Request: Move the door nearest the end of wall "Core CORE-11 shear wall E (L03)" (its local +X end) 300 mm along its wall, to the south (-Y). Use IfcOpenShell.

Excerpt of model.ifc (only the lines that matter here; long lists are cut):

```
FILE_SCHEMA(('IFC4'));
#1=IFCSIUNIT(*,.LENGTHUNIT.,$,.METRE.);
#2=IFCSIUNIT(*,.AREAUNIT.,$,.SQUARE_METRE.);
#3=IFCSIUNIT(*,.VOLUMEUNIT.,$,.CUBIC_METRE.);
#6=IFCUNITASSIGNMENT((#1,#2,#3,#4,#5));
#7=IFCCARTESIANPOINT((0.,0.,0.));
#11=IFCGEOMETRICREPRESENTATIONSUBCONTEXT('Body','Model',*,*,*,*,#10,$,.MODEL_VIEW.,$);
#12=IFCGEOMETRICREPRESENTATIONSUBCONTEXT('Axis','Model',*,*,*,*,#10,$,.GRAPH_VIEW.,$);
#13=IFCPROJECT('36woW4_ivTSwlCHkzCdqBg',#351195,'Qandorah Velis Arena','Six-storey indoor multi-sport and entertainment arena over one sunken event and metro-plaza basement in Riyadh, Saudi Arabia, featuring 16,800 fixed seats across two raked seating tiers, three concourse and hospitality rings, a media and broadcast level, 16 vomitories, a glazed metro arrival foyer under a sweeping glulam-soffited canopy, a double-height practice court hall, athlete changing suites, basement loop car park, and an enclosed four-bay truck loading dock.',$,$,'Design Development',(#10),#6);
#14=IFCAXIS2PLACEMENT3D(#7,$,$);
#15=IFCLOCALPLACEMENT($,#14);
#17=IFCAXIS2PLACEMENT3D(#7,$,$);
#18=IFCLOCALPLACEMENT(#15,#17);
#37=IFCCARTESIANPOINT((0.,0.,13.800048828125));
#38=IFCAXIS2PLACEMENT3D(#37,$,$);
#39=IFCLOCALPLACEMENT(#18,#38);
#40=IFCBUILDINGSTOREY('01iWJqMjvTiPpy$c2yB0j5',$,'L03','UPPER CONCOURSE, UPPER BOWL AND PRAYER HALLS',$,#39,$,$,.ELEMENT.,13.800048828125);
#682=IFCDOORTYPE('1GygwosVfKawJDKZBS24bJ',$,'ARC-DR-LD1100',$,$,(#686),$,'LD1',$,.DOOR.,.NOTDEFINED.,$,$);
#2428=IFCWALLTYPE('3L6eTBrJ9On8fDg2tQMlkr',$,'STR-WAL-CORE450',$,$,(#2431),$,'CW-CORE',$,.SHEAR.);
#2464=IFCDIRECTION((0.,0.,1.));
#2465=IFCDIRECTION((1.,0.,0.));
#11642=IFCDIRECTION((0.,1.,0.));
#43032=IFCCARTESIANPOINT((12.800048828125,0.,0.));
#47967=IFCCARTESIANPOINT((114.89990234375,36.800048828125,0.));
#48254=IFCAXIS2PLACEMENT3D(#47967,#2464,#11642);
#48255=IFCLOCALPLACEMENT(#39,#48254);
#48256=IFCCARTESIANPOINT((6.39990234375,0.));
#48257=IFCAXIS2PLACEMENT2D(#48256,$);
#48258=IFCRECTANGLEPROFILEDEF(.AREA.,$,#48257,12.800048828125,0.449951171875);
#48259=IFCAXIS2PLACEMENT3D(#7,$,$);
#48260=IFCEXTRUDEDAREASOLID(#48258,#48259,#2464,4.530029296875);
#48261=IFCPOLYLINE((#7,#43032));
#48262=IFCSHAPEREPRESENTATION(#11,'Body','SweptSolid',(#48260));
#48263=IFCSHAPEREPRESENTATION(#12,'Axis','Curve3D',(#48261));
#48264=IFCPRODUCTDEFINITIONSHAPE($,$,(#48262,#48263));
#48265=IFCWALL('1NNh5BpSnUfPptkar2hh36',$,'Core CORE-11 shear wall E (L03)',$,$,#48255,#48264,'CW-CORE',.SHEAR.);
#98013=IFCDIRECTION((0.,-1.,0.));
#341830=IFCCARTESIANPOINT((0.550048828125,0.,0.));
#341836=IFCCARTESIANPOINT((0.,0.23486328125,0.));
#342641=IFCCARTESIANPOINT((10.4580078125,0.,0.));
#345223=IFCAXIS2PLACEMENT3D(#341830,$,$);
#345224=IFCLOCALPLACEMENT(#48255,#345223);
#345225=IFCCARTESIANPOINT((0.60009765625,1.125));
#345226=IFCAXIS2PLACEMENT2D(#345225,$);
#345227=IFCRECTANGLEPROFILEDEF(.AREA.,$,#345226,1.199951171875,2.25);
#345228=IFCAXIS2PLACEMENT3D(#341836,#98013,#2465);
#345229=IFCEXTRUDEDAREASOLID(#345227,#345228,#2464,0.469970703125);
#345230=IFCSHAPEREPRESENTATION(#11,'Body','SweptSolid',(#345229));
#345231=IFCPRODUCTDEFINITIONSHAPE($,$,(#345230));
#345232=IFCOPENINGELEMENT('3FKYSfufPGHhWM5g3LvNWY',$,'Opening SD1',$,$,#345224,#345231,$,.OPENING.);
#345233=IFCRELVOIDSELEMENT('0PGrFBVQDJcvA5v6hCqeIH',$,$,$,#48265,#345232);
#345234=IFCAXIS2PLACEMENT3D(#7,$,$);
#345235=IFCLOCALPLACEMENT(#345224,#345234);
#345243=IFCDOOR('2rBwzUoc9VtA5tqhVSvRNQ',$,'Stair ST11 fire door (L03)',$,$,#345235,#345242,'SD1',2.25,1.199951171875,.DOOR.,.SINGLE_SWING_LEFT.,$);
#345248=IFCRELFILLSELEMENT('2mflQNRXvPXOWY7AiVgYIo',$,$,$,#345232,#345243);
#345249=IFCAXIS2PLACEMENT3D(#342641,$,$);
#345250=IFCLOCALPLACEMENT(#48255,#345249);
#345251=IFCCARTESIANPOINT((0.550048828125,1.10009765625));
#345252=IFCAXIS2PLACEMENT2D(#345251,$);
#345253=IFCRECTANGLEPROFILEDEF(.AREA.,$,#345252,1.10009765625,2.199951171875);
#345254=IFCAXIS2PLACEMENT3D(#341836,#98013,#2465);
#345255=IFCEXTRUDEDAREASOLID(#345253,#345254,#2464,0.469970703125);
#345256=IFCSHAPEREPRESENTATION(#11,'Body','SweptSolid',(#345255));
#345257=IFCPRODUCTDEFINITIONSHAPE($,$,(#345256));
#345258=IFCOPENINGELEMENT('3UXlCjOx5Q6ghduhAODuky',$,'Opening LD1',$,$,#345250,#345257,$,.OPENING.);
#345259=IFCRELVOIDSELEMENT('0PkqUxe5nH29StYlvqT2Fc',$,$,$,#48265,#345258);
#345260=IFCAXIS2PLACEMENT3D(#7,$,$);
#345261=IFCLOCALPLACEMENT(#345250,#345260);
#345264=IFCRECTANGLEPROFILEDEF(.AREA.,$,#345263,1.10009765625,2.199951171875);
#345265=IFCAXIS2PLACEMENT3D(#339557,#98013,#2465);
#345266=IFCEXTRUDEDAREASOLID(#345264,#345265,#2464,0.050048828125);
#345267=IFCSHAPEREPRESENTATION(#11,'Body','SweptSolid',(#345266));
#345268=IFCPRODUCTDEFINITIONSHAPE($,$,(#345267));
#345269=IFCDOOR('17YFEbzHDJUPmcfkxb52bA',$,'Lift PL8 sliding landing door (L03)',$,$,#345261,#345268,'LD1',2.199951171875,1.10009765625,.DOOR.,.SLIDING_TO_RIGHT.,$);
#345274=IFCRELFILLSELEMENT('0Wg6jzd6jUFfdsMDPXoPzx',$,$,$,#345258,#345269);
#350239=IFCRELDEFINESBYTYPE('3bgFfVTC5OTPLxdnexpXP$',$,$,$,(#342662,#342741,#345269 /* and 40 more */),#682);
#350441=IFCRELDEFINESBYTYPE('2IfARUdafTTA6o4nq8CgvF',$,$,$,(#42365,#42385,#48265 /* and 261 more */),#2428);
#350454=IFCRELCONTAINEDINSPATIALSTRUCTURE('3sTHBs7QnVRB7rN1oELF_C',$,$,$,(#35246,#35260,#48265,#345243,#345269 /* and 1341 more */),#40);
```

```python
import ifcopenshell
import ifcopenshell.api.geometry
import ifcopenshell.util.placement

model = ifcopenshell.open("model.ifc")

door = model.by_id(345269)
opening = door.FillsVoids[0].RelatingOpeningElement
wall = opening.VoidsElements[0].RelatingBuildingElement

wall_matrix = ifcopenshell.util.placement.get_local_placement(wall.ObjectPlacement)
shift = wall_matrix[:3, 0] * -0.3
before = ifcopenshell.util.placement.get_local_placement(door.ObjectPlacement)[:3, 3].copy()

# The door is placed relative to its opening, so it follows when the opening moves.
matrix = ifcopenshell.util.placement.get_local_placement(opening.ObjectPlacement)
matrix[:3, 3] += shift
ifcopenshell.api.geometry.edit_object_placement(
    model, product=opening, matrix=matrix, is_si=False, should_transform_children=True
)

after = ifcopenshell.util.placement.get_local_placement(door.ObjectPlacement)[:3, 3]
print("door moved by", (after - before).round(3) + 0.0)

model.write("model-out.ifc")
```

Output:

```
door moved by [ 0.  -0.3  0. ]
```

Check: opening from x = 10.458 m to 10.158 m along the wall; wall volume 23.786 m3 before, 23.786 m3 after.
